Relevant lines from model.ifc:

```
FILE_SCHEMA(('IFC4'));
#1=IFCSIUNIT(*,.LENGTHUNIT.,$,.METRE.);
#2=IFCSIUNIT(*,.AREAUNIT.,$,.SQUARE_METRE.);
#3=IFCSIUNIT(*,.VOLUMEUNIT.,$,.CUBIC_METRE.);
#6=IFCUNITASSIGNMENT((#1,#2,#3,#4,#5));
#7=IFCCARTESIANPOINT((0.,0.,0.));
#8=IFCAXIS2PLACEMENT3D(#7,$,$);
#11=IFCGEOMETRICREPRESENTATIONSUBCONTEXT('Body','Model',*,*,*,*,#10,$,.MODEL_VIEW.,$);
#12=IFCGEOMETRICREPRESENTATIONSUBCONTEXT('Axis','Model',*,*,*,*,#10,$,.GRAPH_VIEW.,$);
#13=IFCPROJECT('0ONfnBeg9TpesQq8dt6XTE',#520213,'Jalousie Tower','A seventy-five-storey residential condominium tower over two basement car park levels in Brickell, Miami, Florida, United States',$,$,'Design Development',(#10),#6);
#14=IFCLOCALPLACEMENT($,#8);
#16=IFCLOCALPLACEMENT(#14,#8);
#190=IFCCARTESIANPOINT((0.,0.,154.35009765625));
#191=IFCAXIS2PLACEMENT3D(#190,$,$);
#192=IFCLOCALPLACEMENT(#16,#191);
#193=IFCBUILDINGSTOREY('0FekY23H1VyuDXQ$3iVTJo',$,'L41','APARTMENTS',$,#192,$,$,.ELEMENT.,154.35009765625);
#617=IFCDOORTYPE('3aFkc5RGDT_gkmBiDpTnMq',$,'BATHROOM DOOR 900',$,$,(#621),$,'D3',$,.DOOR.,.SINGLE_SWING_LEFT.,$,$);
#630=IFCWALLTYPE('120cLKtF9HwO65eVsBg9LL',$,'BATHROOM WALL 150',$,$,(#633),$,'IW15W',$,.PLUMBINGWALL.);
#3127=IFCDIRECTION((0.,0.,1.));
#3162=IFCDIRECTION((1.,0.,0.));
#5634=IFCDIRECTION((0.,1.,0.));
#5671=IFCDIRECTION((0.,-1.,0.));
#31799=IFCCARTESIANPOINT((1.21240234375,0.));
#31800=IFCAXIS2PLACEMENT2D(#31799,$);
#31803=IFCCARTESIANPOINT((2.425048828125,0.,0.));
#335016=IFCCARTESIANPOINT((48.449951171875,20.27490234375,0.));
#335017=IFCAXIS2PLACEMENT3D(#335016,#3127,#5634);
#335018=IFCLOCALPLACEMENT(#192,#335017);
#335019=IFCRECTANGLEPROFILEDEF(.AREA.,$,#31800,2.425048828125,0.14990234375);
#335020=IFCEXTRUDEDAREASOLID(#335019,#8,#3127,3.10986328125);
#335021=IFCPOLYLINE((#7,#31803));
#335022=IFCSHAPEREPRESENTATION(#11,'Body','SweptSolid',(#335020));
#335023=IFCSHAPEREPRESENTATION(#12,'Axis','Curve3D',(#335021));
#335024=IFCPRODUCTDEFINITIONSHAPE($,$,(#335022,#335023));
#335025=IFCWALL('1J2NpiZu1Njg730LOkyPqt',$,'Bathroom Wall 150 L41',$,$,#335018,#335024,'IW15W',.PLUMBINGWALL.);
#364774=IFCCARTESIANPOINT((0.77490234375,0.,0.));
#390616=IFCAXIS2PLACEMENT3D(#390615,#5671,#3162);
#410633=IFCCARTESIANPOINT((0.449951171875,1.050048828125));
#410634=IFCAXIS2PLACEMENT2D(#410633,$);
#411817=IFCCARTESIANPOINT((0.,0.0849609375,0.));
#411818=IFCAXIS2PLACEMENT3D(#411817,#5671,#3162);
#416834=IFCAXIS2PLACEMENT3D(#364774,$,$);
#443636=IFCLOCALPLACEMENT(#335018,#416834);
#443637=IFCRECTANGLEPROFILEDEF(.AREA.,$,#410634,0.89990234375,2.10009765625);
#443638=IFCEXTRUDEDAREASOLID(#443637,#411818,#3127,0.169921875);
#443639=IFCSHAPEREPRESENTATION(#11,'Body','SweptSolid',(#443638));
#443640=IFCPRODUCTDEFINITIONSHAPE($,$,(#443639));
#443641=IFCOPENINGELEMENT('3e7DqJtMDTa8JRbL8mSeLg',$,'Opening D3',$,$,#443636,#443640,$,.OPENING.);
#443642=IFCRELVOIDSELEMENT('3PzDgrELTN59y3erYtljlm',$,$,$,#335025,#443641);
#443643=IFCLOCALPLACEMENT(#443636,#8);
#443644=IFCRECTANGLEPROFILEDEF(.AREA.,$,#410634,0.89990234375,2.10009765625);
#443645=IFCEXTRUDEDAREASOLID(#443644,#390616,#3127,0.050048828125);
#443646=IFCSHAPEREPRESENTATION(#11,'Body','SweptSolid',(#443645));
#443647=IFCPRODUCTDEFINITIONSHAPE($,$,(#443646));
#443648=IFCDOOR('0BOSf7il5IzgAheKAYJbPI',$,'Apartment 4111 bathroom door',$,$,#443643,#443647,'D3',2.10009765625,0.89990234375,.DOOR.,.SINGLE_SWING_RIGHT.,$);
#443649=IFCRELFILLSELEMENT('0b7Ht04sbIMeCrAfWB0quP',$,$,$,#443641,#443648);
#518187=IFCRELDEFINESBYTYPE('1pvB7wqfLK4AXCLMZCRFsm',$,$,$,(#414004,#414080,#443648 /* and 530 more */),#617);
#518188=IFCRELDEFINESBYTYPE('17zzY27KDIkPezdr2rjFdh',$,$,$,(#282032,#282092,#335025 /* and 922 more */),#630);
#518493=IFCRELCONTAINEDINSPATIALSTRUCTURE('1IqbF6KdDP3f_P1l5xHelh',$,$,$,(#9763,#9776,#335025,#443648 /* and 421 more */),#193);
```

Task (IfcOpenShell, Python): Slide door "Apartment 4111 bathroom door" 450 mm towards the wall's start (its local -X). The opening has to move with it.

```python
import ifcopenshell
import ifcopenshell.api.geometry
import ifcopenshell.util.placement
import ifcopenshell.util.unit

model = ifcopenshell.open("model.ifc")
unit_scale = ifcopenshell.util.unit.calculate_unit_scale(model)

door = model.by_guid("0BOSf7il5IzgAheKAYJbPI")
opening = door.FillsVoids[0].RelatingOpeningElement
wall = opening.VoidsElements[0].RelatingBuildingElement

wall_matrix = ifcopenshell.util.placement.get_local_placement(wall.ObjectPlacement)
shift = wall_matrix[:3, 0] * -0.45 / unit_scale
before = ifcopenshell.util.placement.get_local_placement(door.ObjectPlacement)[:3, 3].copy()

# The door is placed relative to its opening, so it follows when the opening moves.
matrix = ifcopenshell.util.placement.get_local_placement(opening.ObjectPlacement)
matrix[:3, 3] += shift
ifcopenshell.api.geometry.edit_object_placement(
    model, product=opening, matrix=matrix, is_si=False, should_transform_children=True
)

after = ifcopenshell.util.placement.get_local_placement(door.ObjectPlacement)[:3, 3]
print("door moved by", (after - before).round(3) + 0.0)

model.write("model_v2.ifc")
```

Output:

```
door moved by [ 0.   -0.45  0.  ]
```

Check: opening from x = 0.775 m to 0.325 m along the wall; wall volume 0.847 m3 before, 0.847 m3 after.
